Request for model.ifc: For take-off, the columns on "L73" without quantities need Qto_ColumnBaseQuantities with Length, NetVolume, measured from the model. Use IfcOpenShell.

First a look at what the model holds.

```python
import ifcopenshell
import ifcopenshell.util.element
import ifcopenshell.util.unit

model = ifcopenshell.open("model.ifc")
print(model.schema)
for unit_type in ("LENGTHUNIT", "AREAUNIT", "VOLUMEUNIT"):
    print(unit_type, ifcopenshell.util.unit.calculate_unit_scale(model, unit_type))
storey = next(s for s in model.by_type("IfcBuildingStorey") if s.Name == "L73")
columns = [e for e in ifcopenshell.util.element.get_decomposition(storey) if e.is_a("IfcColumn")]
for e in sorted(columns, key=lambda e: e.id()):
    print(e.id(), e.is_a(), e.Name, list(ifcopenshell.util.element.get_psets(e, qtos_only=True)), sep=" | ")
```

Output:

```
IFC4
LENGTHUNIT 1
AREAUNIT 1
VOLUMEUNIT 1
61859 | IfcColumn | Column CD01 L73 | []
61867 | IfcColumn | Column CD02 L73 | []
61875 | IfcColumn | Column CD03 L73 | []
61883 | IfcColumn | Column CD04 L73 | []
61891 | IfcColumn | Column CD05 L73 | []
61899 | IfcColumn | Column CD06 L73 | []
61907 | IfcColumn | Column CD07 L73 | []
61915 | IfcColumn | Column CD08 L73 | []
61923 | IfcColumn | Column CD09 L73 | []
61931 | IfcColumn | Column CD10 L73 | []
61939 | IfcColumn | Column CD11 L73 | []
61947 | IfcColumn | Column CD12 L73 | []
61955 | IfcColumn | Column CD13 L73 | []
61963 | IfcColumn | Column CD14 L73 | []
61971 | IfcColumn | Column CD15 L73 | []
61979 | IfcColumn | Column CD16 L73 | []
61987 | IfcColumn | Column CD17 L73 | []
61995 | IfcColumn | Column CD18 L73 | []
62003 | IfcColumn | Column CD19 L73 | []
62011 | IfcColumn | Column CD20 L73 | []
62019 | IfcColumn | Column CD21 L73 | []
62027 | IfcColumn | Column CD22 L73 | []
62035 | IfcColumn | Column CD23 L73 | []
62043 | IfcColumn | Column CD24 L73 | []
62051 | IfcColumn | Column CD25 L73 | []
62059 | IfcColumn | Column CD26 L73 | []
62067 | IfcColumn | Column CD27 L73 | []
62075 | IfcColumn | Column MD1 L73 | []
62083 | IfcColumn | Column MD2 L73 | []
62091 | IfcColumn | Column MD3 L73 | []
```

```python
import ifcopenshell
import ifcopenshell.api.pset
import ifcopenshell.geom
import ifcopenshell.util.element
import ifcopenshell.util.shape
import ifcopenshell.util.unit

model = ifcopenshell.open("model.ifc")
unit_scale = ifcopenshell.util.unit.calculate_unit_scale(model)
volume_scale = ifcopenshell.util.unit.calculate_unit_scale(model, "VOLUMEUNIT")
settings = ifcopenshell.geom.settings()

storey = next(s for s in model.by_type("IfcBuildingStorey") if s.Name == "L73")
columns = [e for e in ifcopenshell.util.element.get_decomposition(storey) if e.is_a("IfcColumn")]

for e in sorted(columns, key=lambda e: e.id()):
    if ifcopenshell.util.element.get_psets(e, qtos_only=True, should_inherit=False):
        continue
    # Geometry comes back in metres, in the element's own axes.
    shape = ifcopenshell.geom.create_shape(settings, e)
    values = {
        "Length": ifcopenshell.util.shape.get_z(shape.geometry) / unit_scale,
        "NetVolume": ifcopenshell.util.shape.get_volume(shape.geometry) / volume_scale,
    }
    qto = ifcopenshell.api.pset.add_qto(model, product=e, name="Qto_ColumnBaseQuantities")
    ifcopenshell.api.pset.edit_qto(model, qto=qto, properties=values)
    print(e.id(), {k: round(v, 3) for k, v in values.items()})

model.write("model_edited.ifc")
```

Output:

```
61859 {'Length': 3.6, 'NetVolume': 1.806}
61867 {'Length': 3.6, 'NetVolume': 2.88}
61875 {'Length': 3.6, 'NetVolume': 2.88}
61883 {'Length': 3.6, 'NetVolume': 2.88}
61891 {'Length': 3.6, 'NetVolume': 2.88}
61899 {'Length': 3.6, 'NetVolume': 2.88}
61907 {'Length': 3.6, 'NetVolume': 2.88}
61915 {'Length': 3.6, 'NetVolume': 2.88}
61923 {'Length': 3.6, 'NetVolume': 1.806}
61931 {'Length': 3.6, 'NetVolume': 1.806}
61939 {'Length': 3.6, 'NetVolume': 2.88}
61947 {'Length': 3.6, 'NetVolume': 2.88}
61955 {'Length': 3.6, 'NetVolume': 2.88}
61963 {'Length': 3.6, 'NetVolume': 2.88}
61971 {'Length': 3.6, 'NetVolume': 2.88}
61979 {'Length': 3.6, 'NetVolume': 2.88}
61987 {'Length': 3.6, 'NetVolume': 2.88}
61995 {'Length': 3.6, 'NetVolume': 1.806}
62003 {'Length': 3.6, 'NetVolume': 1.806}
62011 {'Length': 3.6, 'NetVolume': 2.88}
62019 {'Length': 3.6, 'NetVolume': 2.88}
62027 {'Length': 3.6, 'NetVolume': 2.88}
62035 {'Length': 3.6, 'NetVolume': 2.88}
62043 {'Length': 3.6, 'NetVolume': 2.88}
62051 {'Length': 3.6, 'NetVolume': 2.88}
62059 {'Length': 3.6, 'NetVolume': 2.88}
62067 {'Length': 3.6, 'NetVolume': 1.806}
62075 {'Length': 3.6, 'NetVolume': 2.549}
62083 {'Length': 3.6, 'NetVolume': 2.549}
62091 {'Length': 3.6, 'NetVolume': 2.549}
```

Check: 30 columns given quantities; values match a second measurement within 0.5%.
